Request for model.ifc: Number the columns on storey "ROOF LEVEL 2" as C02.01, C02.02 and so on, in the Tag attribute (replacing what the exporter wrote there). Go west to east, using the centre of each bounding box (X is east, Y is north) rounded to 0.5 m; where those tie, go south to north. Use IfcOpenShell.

First a look at what the model holds.

```python
import ifcopenshell
import ifcopenshell.util.element
import ifcopenshell.util.placement

model = ifcopenshell.open("model.ifc")
print(model.schema)
storey = next(s for s in model.by_type("IfcBuildingStorey") if s.Name == "ROOF LEVEL 2")
columns = [e for e in ifcopenshell.util.element.get_decomposition(storey) if e.is_a("IfcColumn")]
for e in sorted(columns, key=lambda e: e.id()):
    origin = ifcopenshell.util.placement.get_local_placement(e.ObjectPlacement)[:3, 3]
    print(e.id(), e.Tag, e.Name, origin.round(2) + 0.0, sep=" | ")
```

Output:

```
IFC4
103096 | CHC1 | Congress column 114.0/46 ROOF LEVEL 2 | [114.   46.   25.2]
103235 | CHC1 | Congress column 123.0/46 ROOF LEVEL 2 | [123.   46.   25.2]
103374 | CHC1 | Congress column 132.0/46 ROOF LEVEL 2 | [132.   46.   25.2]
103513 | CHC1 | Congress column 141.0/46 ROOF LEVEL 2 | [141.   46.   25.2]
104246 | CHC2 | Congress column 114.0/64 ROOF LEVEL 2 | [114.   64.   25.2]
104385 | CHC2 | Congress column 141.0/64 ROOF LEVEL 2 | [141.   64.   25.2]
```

```python
import ifcopenshell
import ifcopenshell.geom
import ifcopenshell.util.element
import ifcopenshell.util.shape

model = ifcopenshell.open("model.ifc")
settings = ifcopenshell.geom.settings()
settings.set("use-world-coords", True)


def centre(element):
    shape = ifcopenshell.geom.create_shape(settings, element)
    return ifcopenshell.util.shape.get_bbox_centroid(shape.geometry)


storey = next(s for s in model.by_type("IfcBuildingStorey") if s.Name == "ROOF LEVEL 2")
columns = [e for e in ifcopenshell.util.element.get_decomposition(storey) if e.is_a("IfcColumn")]

# Insertion points can sit at a corner or the storey origin, so sort by the geometry (in metres).
centres = {e: centre(e) for e in columns}
columns.sort(key=lambda e: (round(centres[e][0] / 0.5), centres[e][1]))

for i, e in enumerate(columns, start=1):
    number = f"C02.{i:02d}"
    e.Tag = number
    print(e.id(), number)

model.write("model_updated.ifc")
```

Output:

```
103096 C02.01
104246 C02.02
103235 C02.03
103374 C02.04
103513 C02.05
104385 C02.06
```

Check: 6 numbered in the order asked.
